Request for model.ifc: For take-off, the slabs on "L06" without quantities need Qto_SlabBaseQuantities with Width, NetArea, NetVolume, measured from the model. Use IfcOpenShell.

First a look at what the model holds.

```python
import ifcopenshell
import ifcopenshell.util.element
import ifcopenshell.util.unit

model = ifcopenshell.open("model.ifc")
print(model.schema)
for unit_type in ("LENGTHUNIT", "AREAUNIT", "VOLUMEUNIT"):
    print(unit_type, ifcopenshell.util.unit.calculate_unit_scale(model, unit_type))
storey = next(s for s in model.by_type("IfcBuildingStorey") if s.Name == "L06")
slabs = [e for e in ifcopenshell.util.element.get_decomposition(storey) if e.is_a("IfcSlab")]
for e in sorted(slabs, key=lambda e: e.id()):
    print(e.id(), e.is_a(), e.Name, list(ifcopenshell.util.element.get_psets(e, qtos_only=True)), sep=" | ")
```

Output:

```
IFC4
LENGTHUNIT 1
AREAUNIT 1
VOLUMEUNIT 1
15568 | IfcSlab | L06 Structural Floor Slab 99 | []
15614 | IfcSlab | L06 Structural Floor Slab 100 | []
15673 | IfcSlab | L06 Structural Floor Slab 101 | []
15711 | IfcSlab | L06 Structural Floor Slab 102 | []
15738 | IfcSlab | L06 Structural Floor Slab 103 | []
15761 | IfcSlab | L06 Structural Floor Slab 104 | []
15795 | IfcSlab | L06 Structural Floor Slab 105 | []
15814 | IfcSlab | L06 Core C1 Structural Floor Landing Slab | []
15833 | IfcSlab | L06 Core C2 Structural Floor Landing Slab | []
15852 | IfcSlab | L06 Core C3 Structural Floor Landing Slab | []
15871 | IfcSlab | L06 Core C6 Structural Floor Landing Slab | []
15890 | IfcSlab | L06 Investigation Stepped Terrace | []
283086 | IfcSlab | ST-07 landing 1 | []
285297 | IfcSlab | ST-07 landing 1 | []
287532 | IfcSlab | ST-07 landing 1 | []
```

```python
import ifcopenshell
import ifcopenshell.api.pset
import ifcopenshell.geom
import ifcopenshell.util.element
import ifcopenshell.util.shape
import ifcopenshell.util.unit

model = ifcopenshell.open("model.ifc")
unit_scale = ifcopenshell.util.unit.calculate_unit_scale(model)
area_scale = ifcopenshell.util.unit.calculate_unit_scale(model, "AREAUNIT")
volume_scale = ifcopenshell.util.unit.calculate_unit_scale(model, "VOLUMEUNIT")
settings = ifcopenshell.geom.settings()

storey = next(s for s in model.by_type("IfcBuildingStorey") if s.Name == "L06")
slabs = [e for e in ifcopenshell.util.element.get_decomposition(storey) if e.is_a("IfcSlab")]

for e in sorted(slabs, key=lambda e: e.id()):
    if ifcopenshell.util.element.get_psets(e, qtos_only=True, should_inherit=False):
        continue
    # Geometry comes back in metres, in the element's own axes.
    shape = ifcopenshell.geom.create_shape(settings, e)
    values = {
        "Width": ifcopenshell.util.shape.get_z(shape.geometry) / unit_scale,
        "NetArea": ifcopenshell.util.shape.get_footprint_area(shape.geometry) / area_scale,
        "NetVolume": ifcopenshell.util.shape.get_volume(shape.geometry) / volume_scale,
    }
    qto = ifcopenshell.api.pset.add_qto(model, product=e, name="Qto_SlabBaseQuantities")
    ifcopenshell.api.pset.edit_qto(model, qto=qto, properties=values)
    print(e.id(), {k: round(v, 3) for k, v in values.items()})

model.write("model_edited.ifc")
```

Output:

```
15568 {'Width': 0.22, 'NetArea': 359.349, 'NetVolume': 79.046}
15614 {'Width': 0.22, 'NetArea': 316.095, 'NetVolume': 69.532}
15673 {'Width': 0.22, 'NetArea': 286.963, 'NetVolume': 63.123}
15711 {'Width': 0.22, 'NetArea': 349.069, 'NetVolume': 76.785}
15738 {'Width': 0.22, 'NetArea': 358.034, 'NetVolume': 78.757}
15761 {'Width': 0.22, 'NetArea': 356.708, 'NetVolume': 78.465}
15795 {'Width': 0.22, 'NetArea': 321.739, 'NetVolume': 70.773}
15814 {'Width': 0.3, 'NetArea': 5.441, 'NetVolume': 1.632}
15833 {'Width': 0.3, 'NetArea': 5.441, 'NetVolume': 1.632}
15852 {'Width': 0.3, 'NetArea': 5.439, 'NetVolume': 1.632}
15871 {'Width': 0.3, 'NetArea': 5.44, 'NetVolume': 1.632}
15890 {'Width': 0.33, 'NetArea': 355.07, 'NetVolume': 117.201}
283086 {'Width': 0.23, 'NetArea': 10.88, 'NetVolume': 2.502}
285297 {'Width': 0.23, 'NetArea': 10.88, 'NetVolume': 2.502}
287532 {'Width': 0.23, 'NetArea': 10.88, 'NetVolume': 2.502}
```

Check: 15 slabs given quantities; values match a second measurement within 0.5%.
